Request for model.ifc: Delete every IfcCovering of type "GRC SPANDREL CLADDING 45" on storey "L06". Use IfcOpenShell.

First a look at what the model holds.

```python
import ifcopenshell
import ifcopenshell.util.element

model = ifcopenshell.open("model.ifc")
print(model.schema)
storey = next(s for s in model.by_type("IfcBuildingStorey") if s.Name == "L06")
coverings = [e for e in ifcopenshell.util.element.get_decomposition(storey) if e.is_a("IfcCovering")]
seen = {}
for e in coverings:
    element_type = ifcopenshell.util.element.get_type(e)
    name = element_type.Name if element_type not in (None, e) else None
    seen[name] = seen.get(name, 0) + 1
for name, count in sorted(seen.items(), key=str):
    print(count, "x", name)
```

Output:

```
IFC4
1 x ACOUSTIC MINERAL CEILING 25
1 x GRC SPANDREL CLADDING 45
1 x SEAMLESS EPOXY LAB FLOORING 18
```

```python
import ifcopenshell
import ifcopenshell.api.root
import ifcopenshell.util.element

model = ifcopenshell.open("model.ifc")

storey = next(s for s in model.by_type("IfcBuildingStorey") if s.Name == "L06")
coverings = [e for e in ifcopenshell.util.element.get_decomposition(storey) if e.is_a("IfcCovering")]
targets = [e for e in coverings if (t := ifcopenshell.util.element.get_type(e)) not in (None, e) and t.Name == "GRC SPANDREL CLADDING 45"]

for e in targets:
    ifcopenshell.api.root.remove_product(model, product=e)
print(len(targets), "removed")

model.write("model-out.ifc")
```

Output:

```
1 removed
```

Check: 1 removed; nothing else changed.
